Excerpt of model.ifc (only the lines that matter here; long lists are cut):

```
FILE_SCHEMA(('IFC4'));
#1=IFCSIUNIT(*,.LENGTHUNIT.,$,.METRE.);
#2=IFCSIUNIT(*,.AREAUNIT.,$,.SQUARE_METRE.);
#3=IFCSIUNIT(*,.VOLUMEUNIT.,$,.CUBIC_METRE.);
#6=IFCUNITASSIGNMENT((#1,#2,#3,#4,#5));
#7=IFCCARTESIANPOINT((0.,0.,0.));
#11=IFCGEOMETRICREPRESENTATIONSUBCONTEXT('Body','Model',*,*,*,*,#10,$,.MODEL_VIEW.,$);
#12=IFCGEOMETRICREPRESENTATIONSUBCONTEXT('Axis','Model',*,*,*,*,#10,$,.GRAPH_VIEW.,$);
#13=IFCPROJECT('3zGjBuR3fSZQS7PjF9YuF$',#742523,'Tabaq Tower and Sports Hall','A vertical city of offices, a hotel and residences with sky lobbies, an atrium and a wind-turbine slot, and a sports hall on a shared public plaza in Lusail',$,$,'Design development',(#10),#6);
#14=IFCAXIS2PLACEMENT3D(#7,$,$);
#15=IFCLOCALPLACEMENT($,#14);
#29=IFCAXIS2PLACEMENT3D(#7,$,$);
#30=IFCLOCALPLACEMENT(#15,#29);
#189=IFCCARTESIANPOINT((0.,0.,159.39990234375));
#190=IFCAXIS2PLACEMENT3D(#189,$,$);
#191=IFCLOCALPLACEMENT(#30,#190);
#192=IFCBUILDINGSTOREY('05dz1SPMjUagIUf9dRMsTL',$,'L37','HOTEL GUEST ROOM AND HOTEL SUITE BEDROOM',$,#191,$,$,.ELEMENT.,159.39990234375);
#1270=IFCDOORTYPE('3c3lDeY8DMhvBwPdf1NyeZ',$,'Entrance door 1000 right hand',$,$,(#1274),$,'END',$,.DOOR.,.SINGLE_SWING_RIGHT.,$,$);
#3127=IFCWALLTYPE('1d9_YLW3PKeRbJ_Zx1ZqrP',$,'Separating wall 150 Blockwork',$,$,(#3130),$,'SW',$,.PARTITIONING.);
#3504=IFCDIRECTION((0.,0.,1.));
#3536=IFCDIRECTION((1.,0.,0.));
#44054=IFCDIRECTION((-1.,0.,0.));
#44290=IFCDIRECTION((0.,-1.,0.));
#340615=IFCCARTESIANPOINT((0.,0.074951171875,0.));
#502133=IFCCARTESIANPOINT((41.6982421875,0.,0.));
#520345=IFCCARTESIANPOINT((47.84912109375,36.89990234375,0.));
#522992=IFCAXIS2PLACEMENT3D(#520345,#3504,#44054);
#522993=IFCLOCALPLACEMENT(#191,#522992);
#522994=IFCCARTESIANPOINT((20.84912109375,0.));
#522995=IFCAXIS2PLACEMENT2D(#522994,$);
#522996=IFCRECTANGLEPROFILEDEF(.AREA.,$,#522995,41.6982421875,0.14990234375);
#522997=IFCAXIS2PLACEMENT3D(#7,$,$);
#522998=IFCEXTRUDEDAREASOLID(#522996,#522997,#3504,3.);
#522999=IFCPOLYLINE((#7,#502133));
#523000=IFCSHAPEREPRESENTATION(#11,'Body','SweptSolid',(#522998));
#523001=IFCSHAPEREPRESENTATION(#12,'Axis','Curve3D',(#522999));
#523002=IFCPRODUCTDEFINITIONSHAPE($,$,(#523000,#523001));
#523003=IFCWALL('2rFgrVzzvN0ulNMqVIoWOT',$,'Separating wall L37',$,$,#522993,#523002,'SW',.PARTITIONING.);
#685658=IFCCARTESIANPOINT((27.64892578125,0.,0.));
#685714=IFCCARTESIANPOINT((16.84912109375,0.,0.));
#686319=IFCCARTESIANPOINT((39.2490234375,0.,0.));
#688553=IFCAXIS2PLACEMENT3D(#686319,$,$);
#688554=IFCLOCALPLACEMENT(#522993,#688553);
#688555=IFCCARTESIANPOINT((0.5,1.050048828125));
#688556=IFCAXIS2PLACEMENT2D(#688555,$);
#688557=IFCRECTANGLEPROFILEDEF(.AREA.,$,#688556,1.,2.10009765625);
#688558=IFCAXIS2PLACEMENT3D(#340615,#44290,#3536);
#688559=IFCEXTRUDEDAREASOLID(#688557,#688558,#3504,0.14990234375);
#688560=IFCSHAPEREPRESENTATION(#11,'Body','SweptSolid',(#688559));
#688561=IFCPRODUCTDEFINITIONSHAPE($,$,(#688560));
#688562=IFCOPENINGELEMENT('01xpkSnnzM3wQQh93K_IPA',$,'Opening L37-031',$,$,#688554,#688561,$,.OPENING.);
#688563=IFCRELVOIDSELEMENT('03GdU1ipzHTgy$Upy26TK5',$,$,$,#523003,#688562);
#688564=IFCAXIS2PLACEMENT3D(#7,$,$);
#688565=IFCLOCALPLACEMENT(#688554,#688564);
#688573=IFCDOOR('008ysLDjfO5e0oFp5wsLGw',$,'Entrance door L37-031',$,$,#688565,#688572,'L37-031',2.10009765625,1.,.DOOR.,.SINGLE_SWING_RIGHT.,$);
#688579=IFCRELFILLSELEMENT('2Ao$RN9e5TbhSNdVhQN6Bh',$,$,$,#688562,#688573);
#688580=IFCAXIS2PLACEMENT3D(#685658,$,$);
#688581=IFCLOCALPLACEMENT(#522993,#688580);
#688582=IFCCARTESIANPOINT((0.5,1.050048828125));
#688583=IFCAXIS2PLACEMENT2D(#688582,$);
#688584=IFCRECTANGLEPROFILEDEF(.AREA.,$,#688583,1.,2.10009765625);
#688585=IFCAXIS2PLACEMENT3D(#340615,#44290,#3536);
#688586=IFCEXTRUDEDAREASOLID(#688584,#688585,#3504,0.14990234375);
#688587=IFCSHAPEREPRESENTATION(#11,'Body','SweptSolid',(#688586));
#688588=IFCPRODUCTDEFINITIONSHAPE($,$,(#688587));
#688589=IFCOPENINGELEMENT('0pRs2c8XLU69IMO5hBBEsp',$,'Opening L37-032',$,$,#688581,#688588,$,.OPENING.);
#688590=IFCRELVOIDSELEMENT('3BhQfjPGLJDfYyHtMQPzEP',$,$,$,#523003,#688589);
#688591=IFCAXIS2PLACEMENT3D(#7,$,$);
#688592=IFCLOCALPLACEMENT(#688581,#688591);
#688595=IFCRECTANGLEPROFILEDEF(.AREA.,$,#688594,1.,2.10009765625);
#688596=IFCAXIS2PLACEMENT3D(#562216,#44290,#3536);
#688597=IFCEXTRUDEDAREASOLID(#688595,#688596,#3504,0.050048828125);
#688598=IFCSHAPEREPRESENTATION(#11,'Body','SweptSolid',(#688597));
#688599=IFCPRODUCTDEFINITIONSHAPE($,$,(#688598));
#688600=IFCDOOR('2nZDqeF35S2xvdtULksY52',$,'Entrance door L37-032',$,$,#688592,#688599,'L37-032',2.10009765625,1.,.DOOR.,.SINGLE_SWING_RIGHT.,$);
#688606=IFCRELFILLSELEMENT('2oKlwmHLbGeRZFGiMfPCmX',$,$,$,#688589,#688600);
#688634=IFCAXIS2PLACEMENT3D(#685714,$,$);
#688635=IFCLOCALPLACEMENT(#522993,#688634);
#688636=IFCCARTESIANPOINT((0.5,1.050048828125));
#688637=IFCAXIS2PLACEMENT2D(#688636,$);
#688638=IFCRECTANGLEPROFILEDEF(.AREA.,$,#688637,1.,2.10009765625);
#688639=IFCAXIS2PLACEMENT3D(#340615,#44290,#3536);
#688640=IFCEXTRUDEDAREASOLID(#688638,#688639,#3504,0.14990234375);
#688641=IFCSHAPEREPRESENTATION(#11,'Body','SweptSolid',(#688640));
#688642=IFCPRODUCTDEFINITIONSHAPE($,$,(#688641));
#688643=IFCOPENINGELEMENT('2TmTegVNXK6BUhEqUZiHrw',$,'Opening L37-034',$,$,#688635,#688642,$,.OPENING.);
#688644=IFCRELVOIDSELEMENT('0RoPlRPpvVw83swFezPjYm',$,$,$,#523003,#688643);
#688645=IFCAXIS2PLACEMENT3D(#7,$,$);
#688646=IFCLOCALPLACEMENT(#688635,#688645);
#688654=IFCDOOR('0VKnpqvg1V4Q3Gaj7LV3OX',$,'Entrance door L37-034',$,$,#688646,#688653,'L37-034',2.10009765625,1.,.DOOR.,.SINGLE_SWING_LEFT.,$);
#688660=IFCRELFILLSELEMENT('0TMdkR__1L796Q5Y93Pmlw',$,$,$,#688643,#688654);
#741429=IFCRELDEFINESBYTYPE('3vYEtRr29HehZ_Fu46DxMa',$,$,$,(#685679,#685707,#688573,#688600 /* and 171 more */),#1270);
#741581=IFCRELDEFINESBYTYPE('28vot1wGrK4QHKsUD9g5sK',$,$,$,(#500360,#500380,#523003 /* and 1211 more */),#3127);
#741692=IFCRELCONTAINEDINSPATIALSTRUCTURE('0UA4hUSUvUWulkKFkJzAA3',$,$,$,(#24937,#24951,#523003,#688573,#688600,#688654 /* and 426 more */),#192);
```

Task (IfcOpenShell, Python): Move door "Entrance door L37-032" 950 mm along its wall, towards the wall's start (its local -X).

```python
import ifcopenshell
import ifcopenshell.api.geometry
import ifcopenshell.util.placement

model = ifcopenshell.open("model.ifc")

door = model.by_guid("2nZDqeF35S2xvdtULksY52")
opening = door.FillsVoids[0].RelatingOpeningElement
wall = opening.VoidsElements[0].RelatingBuildingElement

wall_matrix = ifcopenshell.util.placement.get_local_placement(wall.ObjectPlacement)
shift = wall_matrix[:3, 0] * -0.95
before = ifcopenshell.util.placement.get_local_placement(door.ObjectPlacement)[:3, 3].copy()

# The door is placed relative to its opening, so it follows when the opening moves.
matrix = ifcopenshell.util.placement.get_local_placement(opening.ObjectPlacement)
matrix[:3, 3] += shift
ifcopenshell.api.geometry.edit_object_placement(
    model, product=opening, matrix=matrix, is_si=False, should_transform_children=True
)

after = ifcopenshell.util.placement.get_local_placement(door.ObjectPlacement)[:3, 3]
print("door moved by", (after - before).round(3) + 0.0)

model.write("model_updated.ifc")
```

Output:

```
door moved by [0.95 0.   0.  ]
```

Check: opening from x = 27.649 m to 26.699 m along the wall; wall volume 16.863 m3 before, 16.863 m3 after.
